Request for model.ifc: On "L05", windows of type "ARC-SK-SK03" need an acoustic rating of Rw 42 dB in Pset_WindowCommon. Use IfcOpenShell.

First a look at what the model holds.

```python
import ifcopenshell
import ifcopenshell.util.element

model = ifcopenshell.open("model.ifc")
print(model.schema)
storey = next(s for s in model.by_type("IfcBuildingStorey") if s.Name == "L05")
windows = [e for e in ifcopenshell.util.element.get_decomposition(storey) if e.is_a("IfcWindow")]
seen = {}
for e in windows:
    element_type = ifcopenshell.util.element.get_type(e)
    key = (element_type.Name if element_type != e and element_type else None, ifcopenshell.util.element.get_pset(e, "Pset_WindowCommon", "AcousticRating"))
    seen[key] = seen.get(key, 0) + 1
for (name, value), count in sorted(seen.items(), key=str):
    print(count, "x", name, "|", value)
```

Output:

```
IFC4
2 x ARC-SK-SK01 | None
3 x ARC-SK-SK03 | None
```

```python
import ifcopenshell
import ifcopenshell.api.pset
import ifcopenshell.util.element

model = ifcopenshell.open("model.ifc")

storey = next(s for s in model.by_type("IfcBuildingStorey") if s.Name == "L05")
windows = [e for e in ifcopenshell.util.element.get_decomposition(storey) if e.is_a("IfcWindow")]

count = 0
for e in windows:
    element_type = ifcopenshell.util.element.get_type(e)
    if element_type in (None, e) or element_type.Name != "ARC-SK-SK03":
        continue
    # add_pset returns the element's existing set when there is one.
    pset = ifcopenshell.api.pset.add_pset(model, product=e, name="Pset_WindowCommon")
    ifcopenshell.api.pset.edit_pset(model, pset=pset, properties={"AcousticRating": "Rw 42 dB"})
    count += 1

print(count, "windows updated")

model.write("model_updated.ifc")
```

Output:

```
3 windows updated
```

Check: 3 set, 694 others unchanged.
